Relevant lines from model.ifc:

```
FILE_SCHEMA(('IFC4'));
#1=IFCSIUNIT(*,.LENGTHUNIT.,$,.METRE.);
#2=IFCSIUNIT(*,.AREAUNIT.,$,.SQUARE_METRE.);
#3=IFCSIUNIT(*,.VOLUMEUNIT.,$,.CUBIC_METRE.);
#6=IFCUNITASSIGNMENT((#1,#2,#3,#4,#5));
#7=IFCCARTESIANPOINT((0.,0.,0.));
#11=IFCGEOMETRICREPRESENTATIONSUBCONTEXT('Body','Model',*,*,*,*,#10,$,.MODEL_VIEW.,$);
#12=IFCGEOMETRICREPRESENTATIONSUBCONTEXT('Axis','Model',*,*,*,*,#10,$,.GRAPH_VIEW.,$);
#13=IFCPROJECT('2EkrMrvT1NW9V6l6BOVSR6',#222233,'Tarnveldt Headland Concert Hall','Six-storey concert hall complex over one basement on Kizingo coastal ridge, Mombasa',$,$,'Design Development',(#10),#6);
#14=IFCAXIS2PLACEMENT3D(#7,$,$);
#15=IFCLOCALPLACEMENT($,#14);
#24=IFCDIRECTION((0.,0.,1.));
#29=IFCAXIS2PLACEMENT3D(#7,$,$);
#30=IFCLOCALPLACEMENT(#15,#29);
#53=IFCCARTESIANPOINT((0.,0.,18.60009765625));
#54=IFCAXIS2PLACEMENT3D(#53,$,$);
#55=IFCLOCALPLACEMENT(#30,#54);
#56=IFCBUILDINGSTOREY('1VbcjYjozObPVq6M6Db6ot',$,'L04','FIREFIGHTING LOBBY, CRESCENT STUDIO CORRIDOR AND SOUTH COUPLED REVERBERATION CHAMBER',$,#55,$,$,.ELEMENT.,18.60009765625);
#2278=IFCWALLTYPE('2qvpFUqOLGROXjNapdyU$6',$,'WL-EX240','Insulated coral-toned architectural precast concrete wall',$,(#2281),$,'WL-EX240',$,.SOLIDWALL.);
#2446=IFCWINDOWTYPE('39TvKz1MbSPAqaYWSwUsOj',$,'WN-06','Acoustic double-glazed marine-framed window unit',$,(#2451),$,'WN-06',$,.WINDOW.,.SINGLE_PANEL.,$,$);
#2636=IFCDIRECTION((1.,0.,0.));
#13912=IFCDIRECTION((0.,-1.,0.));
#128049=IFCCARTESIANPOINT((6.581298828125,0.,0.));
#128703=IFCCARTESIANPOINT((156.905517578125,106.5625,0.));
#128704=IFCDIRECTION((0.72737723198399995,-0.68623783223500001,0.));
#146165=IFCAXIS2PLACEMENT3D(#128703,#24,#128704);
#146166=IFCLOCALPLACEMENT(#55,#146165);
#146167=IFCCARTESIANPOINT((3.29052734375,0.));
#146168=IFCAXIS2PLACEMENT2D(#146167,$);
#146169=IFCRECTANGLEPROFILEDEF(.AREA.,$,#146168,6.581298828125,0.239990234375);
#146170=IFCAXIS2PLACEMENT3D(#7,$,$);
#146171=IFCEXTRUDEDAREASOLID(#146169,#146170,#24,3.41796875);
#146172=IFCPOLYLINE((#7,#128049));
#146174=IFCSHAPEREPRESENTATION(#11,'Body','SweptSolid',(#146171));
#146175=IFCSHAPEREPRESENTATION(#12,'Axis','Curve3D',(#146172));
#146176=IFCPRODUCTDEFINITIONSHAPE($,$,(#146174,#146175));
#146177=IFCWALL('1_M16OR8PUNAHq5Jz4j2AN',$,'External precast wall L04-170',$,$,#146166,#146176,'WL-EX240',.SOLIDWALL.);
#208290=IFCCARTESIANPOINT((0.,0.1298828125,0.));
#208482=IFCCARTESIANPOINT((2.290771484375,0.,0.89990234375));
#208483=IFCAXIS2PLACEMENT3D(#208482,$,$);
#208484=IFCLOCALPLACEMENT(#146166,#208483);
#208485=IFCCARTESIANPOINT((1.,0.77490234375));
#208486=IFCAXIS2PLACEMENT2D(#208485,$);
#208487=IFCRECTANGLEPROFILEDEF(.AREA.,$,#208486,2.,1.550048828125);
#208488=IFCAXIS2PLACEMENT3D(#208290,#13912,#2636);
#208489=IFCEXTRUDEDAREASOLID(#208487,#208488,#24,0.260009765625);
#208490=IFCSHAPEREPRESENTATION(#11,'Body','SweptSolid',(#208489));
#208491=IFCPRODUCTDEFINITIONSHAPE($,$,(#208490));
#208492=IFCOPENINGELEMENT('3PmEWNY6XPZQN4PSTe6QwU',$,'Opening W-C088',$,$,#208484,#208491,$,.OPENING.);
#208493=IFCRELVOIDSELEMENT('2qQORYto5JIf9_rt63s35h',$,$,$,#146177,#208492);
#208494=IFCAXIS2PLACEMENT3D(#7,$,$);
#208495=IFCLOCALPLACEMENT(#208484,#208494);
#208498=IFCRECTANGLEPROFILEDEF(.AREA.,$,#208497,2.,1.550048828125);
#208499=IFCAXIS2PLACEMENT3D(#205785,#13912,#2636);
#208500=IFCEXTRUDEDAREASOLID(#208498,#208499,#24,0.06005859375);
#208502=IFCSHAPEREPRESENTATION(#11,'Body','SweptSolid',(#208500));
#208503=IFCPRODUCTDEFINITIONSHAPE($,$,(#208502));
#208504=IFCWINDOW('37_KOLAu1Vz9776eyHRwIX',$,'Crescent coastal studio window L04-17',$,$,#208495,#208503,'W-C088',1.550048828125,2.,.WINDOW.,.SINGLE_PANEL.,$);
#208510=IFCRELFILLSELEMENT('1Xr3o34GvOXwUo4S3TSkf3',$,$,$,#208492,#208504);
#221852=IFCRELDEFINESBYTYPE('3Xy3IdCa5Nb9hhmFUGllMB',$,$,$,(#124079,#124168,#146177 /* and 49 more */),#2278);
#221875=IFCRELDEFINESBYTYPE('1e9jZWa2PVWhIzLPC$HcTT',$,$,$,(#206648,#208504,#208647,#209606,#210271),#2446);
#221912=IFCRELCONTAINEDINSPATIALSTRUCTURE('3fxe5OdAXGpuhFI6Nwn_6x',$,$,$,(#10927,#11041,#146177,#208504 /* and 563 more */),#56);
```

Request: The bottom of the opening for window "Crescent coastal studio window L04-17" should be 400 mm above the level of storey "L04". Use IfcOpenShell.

```python
import numpy as np
import ifcopenshell
import ifcopenshell.api.geometry
import ifcopenshell.geom
import ifcopenshell.util.element
import ifcopenshell.util.placement
import ifcopenshell.util.shape
import ifcopenshell.util.unit

model = ifcopenshell.open("model.ifc")
unit_scale = ifcopenshell.util.unit.calculate_unit_scale(model)

window = model.by_id(208504)
opening = window.FillsVoids[0].RelatingOpeningElement
storey = ifcopenshell.util.element.get_container(window, ifc_class="IfcBuildingStorey")
level = ifcopenshell.util.placement.get_local_placement(storey.ObjectPlacement)[2, 3]

# The opening's origin need not be at the sill, so measure its lowest point.
shape = ifcopenshell.geom.create_shape(ifcopenshell.geom.settings(), opening)
bottom = ifcopenshell.util.shape.get_shape_bottom_elevation(shape, shape.geometry) / unit_scale
dz = level + 0.4 / unit_scale - bottom

shift = np.array([0.0, 0.0, dz])
# The window is placed relative to its opening, so it follows when the opening moves.
matrix = ifcopenshell.util.placement.get_local_placement(opening.ObjectPlacement)
matrix[:3, 3] += shift
ifcopenshell.api.geometry.edit_object_placement(
    model, product=opening, matrix=matrix, is_si=False, should_transform_children=True
)

print(f"moved by {dz * unit_scale:+.3f} m")

model.write("model_rev.ifc")
```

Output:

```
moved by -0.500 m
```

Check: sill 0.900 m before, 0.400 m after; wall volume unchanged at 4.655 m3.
